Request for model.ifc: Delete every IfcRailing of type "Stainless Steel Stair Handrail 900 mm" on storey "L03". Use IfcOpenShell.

First a look at what the model holds.

```python
import ifcopenshell
import ifcopenshell.util.element

model = ifcopenshell.open("model.ifc")
print(model.schema)
storey = next(s for s in model.by_type("IfcBuildingStorey") if s.Name == "L03")
railings = [e for e in ifcopenshell.util.element.get_decomposition(storey) if e.is_a("IfcRailing")]
seen = {}
for e in railings:
    element_type = ifcopenshell.util.element.get_type(e)
    name = element_type.Name if element_type not in (None, e) else None
    seen[name] = seen.get(name, 0) + 1
for name, count in sorted(seen.items(), key=str):
    print(count, "x", name)
```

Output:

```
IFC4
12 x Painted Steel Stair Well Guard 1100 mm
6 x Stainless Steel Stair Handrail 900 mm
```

```python
import ifcopenshell
import ifcopenshell.api.root
import ifcopenshell.util.element

model = ifcopenshell.open("model.ifc")

storey = next(s for s in model.by_type("IfcBuildingStorey") if s.Name == "L03")
railings = [e for e in ifcopenshell.util.element.get_decomposition(storey) if e.is_a("IfcRailing")]
targets = [e for e in railings if (t := ifcopenshell.util.element.get_type(e)) not in (None, e) and t.Name == "Stainless Steel Stair Handrail 900 mm"]

for e in targets:
    ifcopenshell.api.root.remove_product(model, product=e)
print(len(targets), "removed")

model.write("model_updated.ifc")
```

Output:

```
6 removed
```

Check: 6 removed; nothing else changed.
